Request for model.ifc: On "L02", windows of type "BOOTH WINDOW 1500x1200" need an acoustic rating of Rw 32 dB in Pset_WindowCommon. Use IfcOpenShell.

First a look at what the model holds.

```python
import ifcopenshell
import ifcopenshell.util.element

model = ifcopenshell.open("model.ifc")
print(model.schema)
storey = next(s for s in model.by_type("IfcBuildingStorey") if s.Name == "L02")
windows = [e for e in ifcopenshell.util.element.get_decomposition(storey) if e.is_a("IfcWindow")]
seen = {}
for e in windows:
    element_type = ifcopenshell.util.element.get_type(e)
    key = (element_type.Name if element_type != e and element_type else None, ifcopenshell.util.element.get_pset(e, "Pset_WindowCommon", "AcousticRating"))
    seen[key] = seen.get(key, 0) + 1
for (name, value), count in sorted(seen.items(), key=str):
    print(count, "x", name, "|", value)
```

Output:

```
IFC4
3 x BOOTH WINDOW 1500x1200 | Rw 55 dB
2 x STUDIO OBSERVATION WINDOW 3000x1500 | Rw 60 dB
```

```python
import ifcopenshell
import ifcopenshell.api.pset
import ifcopenshell.util.element

model = ifcopenshell.open("model.ifc")

storey = next(s for s in model.by_type("IfcBuildingStorey") if s.Name == "L02")
windows = [e for e in ifcopenshell.util.element.get_decomposition(storey) if e.is_a("IfcWindow")]

count = 0
for e in windows:
    element_type = ifcopenshell.util.element.get_type(e)
    if element_type in (None, e) or element_type.Name != "BOOTH WINDOW 1500x1200":
        continue
    found = ifcopenshell.util.element.get_pset(e, "Pset_WindowCommon", should_inherit=False)
    if found:
        pset = model.by_id(found["id"])
        if len(ifcopenshell.util.element.get_elements_by_pset(pset)) > 1:
            pset = ifcopenshell.api.pset.unshare_pset(model, products=[e], pset=pset)[0]
    else:
        pset = ifcopenshell.api.pset.add_pset(model, product=e, name="Pset_WindowCommon")
    ifcopenshell.api.pset.edit_pset(model, pset=pset, properties={"AcousticRating": "Rw 32 dB"})
    count += 1

print(count, "windows updated")

model.write("model_edited.ifc")
```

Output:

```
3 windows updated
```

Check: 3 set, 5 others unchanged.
